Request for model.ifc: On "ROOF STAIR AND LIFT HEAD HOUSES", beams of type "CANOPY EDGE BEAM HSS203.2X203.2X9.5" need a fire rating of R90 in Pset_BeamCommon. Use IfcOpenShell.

First a look at what the model holds.

```python
import ifcopenshell
import ifcopenshell.util.element

model = ifcopenshell.open("model.ifc")
print(model.schema)
storey = next(s for s in model.by_type("IfcBuildingStorey") if s.Name == "ROOF STAIR AND LIFT HEAD HOUSES")
beams = [e for e in ifcopenshell.util.element.get_decomposition(storey) if e.is_a("IfcBeam")]
seen = {}
for e in beams:
    element_type = ifcopenshell.util.element.get_type(e)
    key = (element_type.Name if element_type != e and element_type else None, ifcopenshell.util.element.get_pset(e, "Pset_BeamCommon", "FireRating"))
    seen[key] = seen.get(key, 0) + 1
for (name, value), count in sorted(seen.items(), key=str):
    print(count, "x", name, "|", value)
```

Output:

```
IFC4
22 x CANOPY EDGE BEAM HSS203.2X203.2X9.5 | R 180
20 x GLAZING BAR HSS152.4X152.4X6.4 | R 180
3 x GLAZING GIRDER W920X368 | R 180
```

```python
import ifcopenshell
import ifcopenshell.api.pset
import ifcopenshell.util.element

model = ifcopenshell.open("model.ifc")

storey = next(s for s in model.by_type("IfcBuildingStorey") if s.Name == "ROOF STAIR AND LIFT HEAD HOUSES")
beams = [e for e in ifcopenshell.util.element.get_decomposition(storey) if e.is_a("IfcBeam")]

count = 0
for e in beams:
    element_type = ifcopenshell.util.element.get_type(e)
    if element_type in (None, e) or element_type.Name != "CANOPY EDGE BEAM HSS203.2X203.2X9.5":
        continue
    found = ifcopenshell.util.element.get_pset(e, "Pset_BeamCommon", should_inherit=False)
    if found:
        pset = model.by_id(found["id"])
        if len(ifcopenshell.util.element.get_elements_by_pset(pset)) > 1:
            pset = ifcopenshell.api.pset.unshare_pset(model, products=[e], pset=pset)[0]
    else:
        pset = ifcopenshell.api.pset.add_pset(model, product=e, name="Pset_BeamCommon")
    ifcopenshell.api.pset.edit_pset(model, pset=pset, properties={"FireRating": "R90"})
    count += 1

print(count, "beams updated")

model.write("model_v2.ifc")
```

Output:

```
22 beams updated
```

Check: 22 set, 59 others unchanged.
